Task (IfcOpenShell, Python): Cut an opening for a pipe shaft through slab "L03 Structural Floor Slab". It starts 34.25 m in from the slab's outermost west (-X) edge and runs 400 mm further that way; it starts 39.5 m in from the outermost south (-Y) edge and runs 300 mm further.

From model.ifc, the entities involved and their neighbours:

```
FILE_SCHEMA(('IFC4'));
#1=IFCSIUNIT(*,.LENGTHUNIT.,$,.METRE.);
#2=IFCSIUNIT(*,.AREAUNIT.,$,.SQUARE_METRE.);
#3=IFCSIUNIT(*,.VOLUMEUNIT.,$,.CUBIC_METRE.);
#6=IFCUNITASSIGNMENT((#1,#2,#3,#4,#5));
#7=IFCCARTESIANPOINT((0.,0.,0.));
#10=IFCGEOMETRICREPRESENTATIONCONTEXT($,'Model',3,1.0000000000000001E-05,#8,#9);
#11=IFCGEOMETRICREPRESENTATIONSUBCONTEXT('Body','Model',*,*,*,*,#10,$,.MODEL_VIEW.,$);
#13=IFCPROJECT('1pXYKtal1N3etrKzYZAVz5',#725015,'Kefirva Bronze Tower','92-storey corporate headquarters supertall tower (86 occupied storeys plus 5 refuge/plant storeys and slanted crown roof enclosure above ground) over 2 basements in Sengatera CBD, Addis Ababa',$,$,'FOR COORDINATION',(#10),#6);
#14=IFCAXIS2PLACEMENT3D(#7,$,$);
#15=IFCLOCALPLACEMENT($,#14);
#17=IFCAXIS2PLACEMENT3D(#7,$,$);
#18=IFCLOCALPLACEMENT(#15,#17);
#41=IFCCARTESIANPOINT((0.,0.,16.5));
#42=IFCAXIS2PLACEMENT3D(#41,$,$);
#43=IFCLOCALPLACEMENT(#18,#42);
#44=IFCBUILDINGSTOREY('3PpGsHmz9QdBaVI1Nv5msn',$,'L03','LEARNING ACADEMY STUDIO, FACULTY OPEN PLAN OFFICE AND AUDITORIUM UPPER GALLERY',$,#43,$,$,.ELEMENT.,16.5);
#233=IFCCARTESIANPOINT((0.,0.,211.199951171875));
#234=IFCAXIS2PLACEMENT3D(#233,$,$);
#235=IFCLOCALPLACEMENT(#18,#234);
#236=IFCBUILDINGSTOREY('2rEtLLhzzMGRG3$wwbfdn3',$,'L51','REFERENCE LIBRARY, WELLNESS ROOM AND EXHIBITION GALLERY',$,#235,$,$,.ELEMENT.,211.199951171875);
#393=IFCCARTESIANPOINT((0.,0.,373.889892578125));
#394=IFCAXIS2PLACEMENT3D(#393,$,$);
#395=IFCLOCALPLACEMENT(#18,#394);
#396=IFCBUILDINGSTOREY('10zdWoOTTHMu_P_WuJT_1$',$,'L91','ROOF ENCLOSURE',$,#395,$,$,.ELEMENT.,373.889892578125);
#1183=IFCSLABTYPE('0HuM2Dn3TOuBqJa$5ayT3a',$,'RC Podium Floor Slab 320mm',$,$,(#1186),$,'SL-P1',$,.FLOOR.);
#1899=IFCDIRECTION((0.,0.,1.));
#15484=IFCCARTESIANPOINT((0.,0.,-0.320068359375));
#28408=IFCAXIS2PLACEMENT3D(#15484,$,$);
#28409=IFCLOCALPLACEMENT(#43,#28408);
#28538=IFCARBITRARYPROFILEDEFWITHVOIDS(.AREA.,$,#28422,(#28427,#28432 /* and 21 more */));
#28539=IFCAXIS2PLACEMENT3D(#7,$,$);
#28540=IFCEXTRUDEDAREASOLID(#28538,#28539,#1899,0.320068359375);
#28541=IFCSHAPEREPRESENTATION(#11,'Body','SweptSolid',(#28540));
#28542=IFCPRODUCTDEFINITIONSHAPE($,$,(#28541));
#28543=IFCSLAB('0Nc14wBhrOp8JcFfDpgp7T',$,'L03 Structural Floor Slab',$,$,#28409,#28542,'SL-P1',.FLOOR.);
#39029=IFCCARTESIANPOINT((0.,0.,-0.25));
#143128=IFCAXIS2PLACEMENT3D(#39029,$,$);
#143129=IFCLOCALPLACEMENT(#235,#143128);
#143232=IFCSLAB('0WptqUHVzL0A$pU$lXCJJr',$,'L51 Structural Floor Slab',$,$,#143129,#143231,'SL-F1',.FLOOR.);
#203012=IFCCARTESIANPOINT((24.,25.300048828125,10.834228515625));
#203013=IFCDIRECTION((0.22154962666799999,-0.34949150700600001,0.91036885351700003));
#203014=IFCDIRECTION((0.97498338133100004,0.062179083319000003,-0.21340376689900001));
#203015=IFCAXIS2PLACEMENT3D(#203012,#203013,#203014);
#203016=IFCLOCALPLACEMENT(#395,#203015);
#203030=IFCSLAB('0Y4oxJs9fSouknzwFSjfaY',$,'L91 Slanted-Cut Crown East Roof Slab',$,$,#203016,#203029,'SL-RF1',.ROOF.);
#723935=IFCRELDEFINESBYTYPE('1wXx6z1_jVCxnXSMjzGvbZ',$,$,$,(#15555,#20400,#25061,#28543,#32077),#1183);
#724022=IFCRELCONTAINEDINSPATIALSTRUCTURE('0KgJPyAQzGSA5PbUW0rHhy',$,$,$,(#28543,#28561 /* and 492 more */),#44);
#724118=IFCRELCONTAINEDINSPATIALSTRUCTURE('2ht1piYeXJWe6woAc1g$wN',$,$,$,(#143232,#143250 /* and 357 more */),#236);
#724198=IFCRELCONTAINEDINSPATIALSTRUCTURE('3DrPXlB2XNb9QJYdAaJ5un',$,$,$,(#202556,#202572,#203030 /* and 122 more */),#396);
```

```python
import numpy as np
import ifcopenshell
import ifcopenshell.api.feature
import ifcopenshell.api.geometry
import ifcopenshell.api.root
import ifcopenshell.geom
import ifcopenshell.util.placement
import ifcopenshell.util.representation
import ifcopenshell.util.shape
import ifcopenshell.util.unit

model = ifcopenshell.open("model.ifc")
unit_scale = ifcopenshell.util.unit.calculate_unit_scale(model)
settings = ifcopenshell.geom.settings()


def volume(element):
    """Net volume in cubic metres, openings subtracted."""
    shape = ifcopenshell.geom.create_shape(settings, element)
    return ifcopenshell.util.shape.get_volume(shape.geometry)


slab = model.by_guid("0Nc14wBhrOp8JcFfDpgp7T")
before = volume(slab)

# Extent in the slab's own axes, in metres. The edges named are its -X and -Y sides.
slab_shape = ifcopenshell.geom.create_shape(settings, slab)
vertices = ifcopenshell.util.shape.get_vertices(slab_shape.geometry)
x_min, y_min, bottom = vertices.min(axis=0)
top = vertices[:, 2].max()

opening = ifcopenshell.api.root.create_entity(model, ifc_class="IfcOpeningElement", name="Pipe shaft opening", predefined_type="OPENING")
context = ifcopenshell.util.representation.get_context(model, "Model", "Body", "MODEL_VIEW")
width, depth = 0.4, 0.3
outline = [(0.0, 0.0), (width, 0.0), (width, depth), (0.0, depth), (0.0, 0.0)]
# Overshoot both faces by 50 mm so the cut is clean.
shape = ifcopenshell.api.geometry.add_slab_representation(
    model, context=context, depth=top - bottom + 0.1, polyline=outline
)
ifcopenshell.api.geometry.assign_representation(model, product=opening, representation=shape)

matrix = ifcopenshell.util.placement.get_local_placement(slab.ObjectPlacement)
matrix[:, 3] = matrix @ np.append(np.array([x_min + 34.25, y_min + 39.5, bottom - 0.05]) / unit_scale, 1.0)
ifcopenshell.api.geometry.edit_object_placement(model, product=opening, matrix=matrix, is_si=False)
ifcopenshell.api.feature.add_feature(model, feature=opening, element=slab)

after = volume(slab)

print(f"slab volume {before:.3f} -> {after:.3f} m3")

model.write("model_rev.ifc")
```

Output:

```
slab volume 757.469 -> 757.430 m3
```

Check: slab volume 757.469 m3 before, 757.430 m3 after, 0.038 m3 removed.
